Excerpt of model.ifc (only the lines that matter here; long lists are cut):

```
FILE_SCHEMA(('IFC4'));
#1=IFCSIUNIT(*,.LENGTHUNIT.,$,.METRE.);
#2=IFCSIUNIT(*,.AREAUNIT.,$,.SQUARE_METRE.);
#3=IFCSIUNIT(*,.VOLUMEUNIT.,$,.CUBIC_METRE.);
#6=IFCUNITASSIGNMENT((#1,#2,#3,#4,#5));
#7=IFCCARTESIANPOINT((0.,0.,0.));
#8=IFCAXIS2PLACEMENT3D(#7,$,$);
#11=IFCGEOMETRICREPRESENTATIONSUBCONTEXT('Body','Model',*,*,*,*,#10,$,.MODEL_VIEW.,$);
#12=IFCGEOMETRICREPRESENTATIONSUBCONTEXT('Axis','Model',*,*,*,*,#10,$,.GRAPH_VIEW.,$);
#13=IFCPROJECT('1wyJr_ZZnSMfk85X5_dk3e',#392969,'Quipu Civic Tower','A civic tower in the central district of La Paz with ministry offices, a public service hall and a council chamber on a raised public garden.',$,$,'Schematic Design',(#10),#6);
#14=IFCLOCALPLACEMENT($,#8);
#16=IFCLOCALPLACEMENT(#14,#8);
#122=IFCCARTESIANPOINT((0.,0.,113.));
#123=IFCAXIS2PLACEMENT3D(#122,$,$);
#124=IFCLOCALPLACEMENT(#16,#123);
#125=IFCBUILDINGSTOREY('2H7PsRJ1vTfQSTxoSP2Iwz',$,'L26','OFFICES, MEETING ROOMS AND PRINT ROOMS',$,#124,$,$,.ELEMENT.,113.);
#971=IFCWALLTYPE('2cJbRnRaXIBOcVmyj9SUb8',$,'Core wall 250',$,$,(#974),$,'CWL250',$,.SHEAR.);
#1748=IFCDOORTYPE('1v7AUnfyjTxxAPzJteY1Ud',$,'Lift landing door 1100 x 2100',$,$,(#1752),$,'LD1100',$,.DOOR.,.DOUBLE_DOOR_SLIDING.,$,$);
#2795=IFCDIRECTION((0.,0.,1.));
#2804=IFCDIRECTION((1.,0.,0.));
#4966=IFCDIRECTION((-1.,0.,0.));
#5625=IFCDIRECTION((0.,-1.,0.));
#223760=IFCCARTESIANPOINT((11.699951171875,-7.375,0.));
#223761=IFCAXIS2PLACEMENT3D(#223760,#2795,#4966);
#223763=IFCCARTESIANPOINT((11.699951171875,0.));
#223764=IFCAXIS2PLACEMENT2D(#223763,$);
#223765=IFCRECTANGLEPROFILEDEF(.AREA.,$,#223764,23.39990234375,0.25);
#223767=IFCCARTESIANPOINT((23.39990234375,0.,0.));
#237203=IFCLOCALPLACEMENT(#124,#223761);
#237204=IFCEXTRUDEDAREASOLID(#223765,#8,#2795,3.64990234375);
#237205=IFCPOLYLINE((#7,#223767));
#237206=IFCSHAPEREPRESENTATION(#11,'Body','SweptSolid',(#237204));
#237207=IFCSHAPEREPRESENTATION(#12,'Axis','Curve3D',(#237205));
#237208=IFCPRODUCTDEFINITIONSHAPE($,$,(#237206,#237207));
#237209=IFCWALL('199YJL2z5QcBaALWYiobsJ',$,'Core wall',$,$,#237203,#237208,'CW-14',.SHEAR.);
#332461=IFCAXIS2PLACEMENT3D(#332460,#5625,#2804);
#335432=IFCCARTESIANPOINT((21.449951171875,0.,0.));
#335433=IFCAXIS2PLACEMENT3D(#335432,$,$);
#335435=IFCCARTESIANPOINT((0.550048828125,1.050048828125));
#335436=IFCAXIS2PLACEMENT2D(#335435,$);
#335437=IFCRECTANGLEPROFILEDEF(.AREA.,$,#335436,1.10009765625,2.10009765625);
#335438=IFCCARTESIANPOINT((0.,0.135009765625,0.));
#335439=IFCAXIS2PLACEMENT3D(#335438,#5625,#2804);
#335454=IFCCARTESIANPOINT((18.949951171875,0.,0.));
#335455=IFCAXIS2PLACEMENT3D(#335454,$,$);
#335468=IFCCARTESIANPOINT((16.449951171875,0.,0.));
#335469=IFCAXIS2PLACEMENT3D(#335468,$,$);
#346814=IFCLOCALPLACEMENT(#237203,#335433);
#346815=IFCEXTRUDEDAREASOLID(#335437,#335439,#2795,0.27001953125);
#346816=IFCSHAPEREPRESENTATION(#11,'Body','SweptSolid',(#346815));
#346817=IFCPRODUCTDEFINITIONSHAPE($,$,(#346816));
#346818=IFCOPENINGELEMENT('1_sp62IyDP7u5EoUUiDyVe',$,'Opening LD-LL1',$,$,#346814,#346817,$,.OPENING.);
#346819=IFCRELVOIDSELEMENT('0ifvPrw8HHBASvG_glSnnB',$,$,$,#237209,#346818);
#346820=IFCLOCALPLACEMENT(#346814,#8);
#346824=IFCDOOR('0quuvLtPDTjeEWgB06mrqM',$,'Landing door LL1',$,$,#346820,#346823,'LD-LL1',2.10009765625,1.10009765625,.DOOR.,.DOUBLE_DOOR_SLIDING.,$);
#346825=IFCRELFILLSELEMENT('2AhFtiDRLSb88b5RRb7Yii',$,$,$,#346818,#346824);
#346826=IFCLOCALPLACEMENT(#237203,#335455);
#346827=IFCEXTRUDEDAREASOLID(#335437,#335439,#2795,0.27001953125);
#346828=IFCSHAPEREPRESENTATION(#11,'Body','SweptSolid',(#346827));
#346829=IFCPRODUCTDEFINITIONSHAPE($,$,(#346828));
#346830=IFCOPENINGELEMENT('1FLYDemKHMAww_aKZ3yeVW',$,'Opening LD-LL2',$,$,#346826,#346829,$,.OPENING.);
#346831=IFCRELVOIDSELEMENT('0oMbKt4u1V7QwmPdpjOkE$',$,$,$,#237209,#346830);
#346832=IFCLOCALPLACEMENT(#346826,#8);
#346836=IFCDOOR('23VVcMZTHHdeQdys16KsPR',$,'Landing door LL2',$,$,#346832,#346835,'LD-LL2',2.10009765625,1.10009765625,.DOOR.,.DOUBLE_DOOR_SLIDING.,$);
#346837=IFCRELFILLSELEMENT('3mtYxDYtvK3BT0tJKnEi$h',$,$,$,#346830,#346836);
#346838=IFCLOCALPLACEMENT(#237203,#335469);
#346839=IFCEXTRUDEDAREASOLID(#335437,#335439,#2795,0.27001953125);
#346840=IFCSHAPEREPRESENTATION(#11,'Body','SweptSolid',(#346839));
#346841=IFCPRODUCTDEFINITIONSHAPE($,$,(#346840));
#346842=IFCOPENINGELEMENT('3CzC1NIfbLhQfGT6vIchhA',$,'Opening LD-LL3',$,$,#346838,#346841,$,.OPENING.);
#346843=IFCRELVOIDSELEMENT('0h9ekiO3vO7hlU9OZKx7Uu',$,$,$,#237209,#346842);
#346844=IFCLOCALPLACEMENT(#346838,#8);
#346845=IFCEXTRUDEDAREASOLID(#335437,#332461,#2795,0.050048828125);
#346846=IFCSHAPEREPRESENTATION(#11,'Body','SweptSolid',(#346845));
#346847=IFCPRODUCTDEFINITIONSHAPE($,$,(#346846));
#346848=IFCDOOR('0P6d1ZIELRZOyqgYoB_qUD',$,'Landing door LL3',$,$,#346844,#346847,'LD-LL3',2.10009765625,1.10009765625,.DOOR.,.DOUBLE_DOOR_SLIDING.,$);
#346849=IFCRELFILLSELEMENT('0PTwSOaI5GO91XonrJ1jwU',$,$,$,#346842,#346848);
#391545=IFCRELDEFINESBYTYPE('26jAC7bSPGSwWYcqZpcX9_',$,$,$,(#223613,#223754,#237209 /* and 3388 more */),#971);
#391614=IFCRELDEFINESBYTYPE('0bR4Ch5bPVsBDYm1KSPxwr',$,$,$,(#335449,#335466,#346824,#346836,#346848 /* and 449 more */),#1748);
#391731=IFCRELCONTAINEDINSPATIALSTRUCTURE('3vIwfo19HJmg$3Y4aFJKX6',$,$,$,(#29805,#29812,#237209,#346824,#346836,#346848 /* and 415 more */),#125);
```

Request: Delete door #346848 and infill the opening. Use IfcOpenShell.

```python
import ifcopenshell
import ifcopenshell.api.feature
import ifcopenshell.api.root
import ifcopenshell.geom
import ifcopenshell.util.shape

model = ifcopenshell.open("model.ifc")
settings = ifcopenshell.geom.settings()


def volume(element):
    """Net volume in cubic metres, openings subtracted."""
    shape = ifcopenshell.geom.create_shape(settings, element)
    return ifcopenshell.util.shape.get_volume(shape.geometry)


door = model.by_guid("0P6d1ZIELRZOyqgYoB_qUD")
opening = door.FillsVoids[0].RelatingOpeningElement
wall = opening.VoidsElements[0].RelatingBuildingElement
before = volume(wall)

ifcopenshell.api.root.remove_product(model, product=door)
ifcopenshell.api.feature.remove_feature(model, feature=opening)

after = volume(wall)

print(f"wall volume {before:.3f} -> {after:.3f} m3")

model.write("model_v2.ifc")
```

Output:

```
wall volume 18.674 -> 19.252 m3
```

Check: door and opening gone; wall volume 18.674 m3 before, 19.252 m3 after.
